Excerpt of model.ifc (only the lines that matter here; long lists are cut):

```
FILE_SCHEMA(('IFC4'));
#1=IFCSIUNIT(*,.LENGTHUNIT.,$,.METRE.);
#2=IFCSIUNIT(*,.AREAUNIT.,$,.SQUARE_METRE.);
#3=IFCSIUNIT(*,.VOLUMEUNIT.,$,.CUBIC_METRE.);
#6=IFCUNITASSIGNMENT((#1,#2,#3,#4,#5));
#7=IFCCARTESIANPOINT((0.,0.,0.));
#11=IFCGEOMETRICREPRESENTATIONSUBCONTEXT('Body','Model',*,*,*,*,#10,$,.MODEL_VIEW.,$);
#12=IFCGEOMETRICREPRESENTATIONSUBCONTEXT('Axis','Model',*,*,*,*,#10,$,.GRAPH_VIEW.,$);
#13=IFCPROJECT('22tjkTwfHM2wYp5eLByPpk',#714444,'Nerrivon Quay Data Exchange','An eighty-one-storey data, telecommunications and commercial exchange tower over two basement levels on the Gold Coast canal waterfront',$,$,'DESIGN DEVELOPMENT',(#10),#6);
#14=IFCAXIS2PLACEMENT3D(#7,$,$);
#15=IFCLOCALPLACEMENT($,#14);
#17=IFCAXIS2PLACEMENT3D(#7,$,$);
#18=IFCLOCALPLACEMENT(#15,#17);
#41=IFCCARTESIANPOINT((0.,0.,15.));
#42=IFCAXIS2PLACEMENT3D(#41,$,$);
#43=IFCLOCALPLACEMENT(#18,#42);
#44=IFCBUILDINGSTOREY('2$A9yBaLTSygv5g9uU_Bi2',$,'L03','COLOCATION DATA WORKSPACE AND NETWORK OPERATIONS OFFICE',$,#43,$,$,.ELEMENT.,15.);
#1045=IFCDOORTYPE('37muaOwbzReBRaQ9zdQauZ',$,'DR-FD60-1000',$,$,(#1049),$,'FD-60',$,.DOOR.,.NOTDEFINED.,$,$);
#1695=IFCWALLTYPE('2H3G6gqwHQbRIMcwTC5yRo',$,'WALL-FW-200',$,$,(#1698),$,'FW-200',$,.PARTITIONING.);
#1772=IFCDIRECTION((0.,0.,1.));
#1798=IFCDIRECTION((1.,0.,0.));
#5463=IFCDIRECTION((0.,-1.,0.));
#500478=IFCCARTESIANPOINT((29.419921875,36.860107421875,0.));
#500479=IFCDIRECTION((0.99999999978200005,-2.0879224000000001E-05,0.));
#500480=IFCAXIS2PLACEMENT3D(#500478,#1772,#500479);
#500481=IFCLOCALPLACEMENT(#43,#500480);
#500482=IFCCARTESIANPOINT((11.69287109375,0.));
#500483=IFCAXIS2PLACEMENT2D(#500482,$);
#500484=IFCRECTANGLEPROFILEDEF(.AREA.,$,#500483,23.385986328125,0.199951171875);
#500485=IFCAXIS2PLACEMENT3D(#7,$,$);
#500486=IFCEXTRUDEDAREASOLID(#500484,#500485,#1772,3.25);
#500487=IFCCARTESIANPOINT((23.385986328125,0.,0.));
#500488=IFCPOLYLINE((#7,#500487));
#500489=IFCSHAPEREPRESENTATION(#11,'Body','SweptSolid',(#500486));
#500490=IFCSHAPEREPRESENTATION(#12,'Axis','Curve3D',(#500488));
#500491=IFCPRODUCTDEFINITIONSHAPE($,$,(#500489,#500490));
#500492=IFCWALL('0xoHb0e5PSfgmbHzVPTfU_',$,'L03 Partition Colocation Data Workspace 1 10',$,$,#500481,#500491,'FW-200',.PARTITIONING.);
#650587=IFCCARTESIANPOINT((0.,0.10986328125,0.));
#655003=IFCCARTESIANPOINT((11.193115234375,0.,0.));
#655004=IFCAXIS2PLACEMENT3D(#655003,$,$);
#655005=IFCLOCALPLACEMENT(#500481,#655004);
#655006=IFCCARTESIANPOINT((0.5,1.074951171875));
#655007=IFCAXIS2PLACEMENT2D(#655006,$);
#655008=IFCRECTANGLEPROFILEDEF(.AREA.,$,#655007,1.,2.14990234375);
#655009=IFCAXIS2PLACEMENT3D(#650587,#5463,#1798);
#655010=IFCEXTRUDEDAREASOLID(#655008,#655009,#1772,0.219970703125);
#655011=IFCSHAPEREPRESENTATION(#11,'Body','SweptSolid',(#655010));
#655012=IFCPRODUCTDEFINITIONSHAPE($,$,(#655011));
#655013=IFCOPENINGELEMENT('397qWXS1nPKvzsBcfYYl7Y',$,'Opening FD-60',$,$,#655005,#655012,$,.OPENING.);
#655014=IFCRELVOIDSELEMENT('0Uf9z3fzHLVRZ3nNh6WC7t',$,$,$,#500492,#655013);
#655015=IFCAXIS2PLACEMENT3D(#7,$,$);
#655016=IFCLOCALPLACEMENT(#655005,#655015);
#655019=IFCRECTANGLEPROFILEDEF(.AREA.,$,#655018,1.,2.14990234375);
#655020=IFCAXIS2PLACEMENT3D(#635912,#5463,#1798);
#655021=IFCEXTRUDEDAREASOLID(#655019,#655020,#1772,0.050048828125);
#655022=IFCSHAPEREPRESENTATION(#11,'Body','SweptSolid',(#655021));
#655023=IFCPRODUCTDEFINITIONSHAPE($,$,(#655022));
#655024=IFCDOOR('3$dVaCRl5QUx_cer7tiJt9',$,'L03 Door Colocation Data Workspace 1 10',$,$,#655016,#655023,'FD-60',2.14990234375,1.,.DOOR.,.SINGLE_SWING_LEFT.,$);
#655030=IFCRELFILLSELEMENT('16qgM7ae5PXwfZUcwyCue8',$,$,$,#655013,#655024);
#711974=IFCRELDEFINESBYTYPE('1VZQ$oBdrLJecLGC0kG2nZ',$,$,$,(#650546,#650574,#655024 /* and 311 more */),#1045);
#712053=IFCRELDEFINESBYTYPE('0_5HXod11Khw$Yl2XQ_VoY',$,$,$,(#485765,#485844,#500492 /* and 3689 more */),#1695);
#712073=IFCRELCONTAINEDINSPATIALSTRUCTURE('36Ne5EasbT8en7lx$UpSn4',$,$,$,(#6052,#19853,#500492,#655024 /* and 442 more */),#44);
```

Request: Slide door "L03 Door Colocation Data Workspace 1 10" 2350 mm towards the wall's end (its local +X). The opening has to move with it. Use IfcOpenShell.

```python
import ifcopenshell
import ifcopenshell.api.geometry
import ifcopenshell.util.placement

model = ifcopenshell.open("model.ifc")

door = model.by_id(655024)
opening = door.FillsVoids[0].RelatingOpeningElement
wall = opening.VoidsElements[0].RelatingBuildingElement

wall_matrix = ifcopenshell.util.placement.get_local_placement(wall.ObjectPlacement)
shift = wall_matrix[:3, 0] * 2.35
before = ifcopenshell.util.placement.get_local_placement(door.ObjectPlacement)[:3, 3].copy()

# The door is placed relative to its opening, so it follows when the opening moves.
matrix = ifcopenshell.util.placement.get_local_placement(opening.ObjectPlacement)
matrix[:3, 3] += shift
ifcopenshell.api.geometry.edit_object_placement(
    model, product=opening, matrix=matrix, is_si=False, should_transform_children=True
)

after = ifcopenshell.util.placement.get_local_placement(door.ObjectPlacement)[:3, 3]
print("door moved by", (after - before).round(3) + 0.0)

model.write("model_updated.ifc")
```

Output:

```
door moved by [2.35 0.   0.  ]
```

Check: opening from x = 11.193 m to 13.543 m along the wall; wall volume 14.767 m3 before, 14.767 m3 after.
